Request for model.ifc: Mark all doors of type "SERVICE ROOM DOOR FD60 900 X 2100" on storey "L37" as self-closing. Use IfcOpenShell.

First a look at what the model holds.

```python
import ifcopenshell
import ifcopenshell.util.element

model = ifcopenshell.open("model.ifc")
print(model.schema)
storey = next(s for s in model.by_type("IfcBuildingStorey") if s.Name == "L37")
doors = [e for e in ifcopenshell.util.element.get_decomposition(storey) if e.is_a("IfcDoor")]
seen = {}
for e in doors:
    element_type = ifcopenshell.util.element.get_type(e)
    key = (element_type.Name if element_type != e and element_type else None, ifcopenshell.util.element.get_pset(e, "Pset_DoorCommon", "SelfClosing"))
    seen[key] = seen.get(key, 0) + 1
for (name, value), count in sorted(seen.items(), key=str):
    print(count, "x", name, "|", value)
```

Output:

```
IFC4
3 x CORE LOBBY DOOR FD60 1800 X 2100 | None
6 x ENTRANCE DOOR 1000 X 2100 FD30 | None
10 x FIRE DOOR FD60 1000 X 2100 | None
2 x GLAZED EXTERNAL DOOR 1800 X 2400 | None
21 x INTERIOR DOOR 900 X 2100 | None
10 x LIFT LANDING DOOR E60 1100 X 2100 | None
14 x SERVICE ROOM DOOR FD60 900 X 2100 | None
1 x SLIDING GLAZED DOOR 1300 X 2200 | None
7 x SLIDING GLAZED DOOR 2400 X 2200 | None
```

```python
import ifcopenshell
import ifcopenshell.api.pset
import ifcopenshell.util.element

model = ifcopenshell.open("model.ifc")

storey = next(s for s in model.by_type("IfcBuildingStorey") if s.Name == "L37")
doors = [e for e in ifcopenshell.util.element.get_decomposition(storey) if e.is_a("IfcDoor")]

count = 0
for e in doors:
    element_type = ifcopenshell.util.element.get_type(e)
    if element_type in (None, e) or element_type.Name != "SERVICE ROOM DOOR FD60 900 X 2100":
        continue
    found = ifcopenshell.util.element.get_pset(e, "Pset_DoorCommon", should_inherit=False)
    if found:
        pset = model.by_id(found["id"])
        if len(ifcopenshell.util.element.get_elements_by_pset(pset)) > 1:
            pset = ifcopenshell.api.pset.unshare_pset(model, products=[e], pset=pset)[0]
    else:
        pset = ifcopenshell.api.pset.add_pset(model, product=e, name="Pset_DoorCommon")
    ifcopenshell.api.pset.edit_pset(model, pset=pset, properties={"SelfClosing": True})
    count += 1

print(count, "doors updated")

model.write("model-out.ifc")
```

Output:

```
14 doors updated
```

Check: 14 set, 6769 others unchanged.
